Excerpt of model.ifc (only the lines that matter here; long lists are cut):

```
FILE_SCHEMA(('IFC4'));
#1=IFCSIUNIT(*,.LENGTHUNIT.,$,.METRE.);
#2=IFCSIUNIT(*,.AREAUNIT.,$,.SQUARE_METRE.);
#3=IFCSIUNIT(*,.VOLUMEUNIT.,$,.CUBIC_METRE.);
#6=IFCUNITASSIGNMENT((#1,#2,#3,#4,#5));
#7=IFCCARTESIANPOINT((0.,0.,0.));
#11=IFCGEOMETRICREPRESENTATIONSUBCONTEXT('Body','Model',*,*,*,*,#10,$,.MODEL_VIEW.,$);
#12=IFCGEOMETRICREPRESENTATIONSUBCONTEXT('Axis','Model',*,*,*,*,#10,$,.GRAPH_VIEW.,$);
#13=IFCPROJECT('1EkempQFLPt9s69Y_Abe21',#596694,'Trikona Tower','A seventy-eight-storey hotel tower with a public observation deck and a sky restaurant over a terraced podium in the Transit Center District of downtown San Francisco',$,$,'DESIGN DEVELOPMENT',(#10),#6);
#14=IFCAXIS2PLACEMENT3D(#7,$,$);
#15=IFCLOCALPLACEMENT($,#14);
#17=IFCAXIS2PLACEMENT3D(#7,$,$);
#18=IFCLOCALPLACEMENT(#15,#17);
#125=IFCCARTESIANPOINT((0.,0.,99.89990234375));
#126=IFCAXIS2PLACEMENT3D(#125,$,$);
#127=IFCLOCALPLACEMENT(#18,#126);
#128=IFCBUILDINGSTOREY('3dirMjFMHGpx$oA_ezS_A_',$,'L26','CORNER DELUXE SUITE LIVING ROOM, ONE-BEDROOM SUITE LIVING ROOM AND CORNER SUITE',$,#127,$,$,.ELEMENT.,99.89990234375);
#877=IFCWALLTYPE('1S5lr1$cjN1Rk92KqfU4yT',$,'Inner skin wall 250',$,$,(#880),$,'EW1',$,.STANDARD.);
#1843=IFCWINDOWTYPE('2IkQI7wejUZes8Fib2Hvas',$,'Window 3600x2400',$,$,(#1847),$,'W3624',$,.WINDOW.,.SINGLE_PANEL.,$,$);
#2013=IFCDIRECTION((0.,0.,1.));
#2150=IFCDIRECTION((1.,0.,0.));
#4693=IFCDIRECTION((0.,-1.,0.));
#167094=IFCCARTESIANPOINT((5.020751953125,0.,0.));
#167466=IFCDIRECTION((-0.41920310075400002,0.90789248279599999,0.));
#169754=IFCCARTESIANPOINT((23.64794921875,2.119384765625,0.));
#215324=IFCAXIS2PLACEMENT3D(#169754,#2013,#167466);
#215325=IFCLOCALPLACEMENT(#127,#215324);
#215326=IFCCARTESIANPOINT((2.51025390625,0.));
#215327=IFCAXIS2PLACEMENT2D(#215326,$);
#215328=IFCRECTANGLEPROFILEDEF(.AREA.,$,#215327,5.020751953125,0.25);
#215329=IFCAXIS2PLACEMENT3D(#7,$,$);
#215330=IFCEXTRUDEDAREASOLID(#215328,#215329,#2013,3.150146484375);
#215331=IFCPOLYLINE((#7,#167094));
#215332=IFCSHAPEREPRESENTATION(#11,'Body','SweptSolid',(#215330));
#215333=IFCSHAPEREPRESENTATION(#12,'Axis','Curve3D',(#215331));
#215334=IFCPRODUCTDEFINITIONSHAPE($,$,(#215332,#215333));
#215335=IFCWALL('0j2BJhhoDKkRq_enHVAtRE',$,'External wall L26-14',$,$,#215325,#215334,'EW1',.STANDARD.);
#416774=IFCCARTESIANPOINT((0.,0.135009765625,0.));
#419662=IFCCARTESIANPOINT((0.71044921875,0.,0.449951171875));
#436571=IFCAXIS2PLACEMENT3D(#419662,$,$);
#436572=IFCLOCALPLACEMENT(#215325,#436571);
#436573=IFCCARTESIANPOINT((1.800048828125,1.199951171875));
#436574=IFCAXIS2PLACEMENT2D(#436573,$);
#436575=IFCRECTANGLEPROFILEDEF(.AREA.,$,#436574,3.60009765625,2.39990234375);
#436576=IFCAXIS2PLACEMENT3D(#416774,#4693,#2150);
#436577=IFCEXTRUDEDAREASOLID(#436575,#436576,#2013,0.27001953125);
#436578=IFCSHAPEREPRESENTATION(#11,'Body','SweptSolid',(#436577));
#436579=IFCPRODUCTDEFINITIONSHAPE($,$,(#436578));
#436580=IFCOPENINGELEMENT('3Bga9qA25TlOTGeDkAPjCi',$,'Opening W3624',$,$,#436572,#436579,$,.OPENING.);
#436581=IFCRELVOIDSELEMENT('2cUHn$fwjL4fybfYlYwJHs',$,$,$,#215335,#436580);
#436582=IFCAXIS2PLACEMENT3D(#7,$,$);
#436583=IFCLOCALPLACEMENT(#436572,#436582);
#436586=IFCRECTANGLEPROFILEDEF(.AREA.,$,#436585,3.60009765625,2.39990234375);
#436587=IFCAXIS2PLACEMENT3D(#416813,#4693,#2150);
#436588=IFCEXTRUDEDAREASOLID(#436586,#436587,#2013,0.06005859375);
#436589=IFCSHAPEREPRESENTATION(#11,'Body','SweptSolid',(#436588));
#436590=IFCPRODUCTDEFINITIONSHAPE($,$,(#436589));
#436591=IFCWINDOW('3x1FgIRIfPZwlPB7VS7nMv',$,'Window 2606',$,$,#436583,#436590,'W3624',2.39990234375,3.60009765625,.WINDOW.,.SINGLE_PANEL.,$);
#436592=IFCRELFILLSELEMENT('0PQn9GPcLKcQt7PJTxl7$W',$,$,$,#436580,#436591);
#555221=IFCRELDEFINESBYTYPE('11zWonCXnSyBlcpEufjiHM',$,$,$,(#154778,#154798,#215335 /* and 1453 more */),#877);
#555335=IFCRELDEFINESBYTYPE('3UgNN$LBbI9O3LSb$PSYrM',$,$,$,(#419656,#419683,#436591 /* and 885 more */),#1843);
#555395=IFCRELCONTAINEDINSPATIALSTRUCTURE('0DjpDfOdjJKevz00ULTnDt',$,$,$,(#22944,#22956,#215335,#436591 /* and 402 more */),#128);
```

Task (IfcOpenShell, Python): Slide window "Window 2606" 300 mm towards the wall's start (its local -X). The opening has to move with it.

```python
import ifcopenshell
import ifcopenshell.api.geometry
import ifcopenshell.util.placement

model = ifcopenshell.open("model.ifc")

window = model.by_guid("3x1FgIRIfPZwlPB7VS7nMv")
opening = window.FillsVoids[0].RelatingOpeningElement
wall = opening.VoidsElements[0].RelatingBuildingElement

wall_matrix = ifcopenshell.util.placement.get_local_placement(wall.ObjectPlacement)
shift = wall_matrix[:3, 0] * -0.3
before = ifcopenshell.util.placement.get_local_placement(window.ObjectPlacement)[:3, 3].copy()

# The window is placed relative to its opening, so it follows when the opening moves.
matrix = ifcopenshell.util.placement.get_local_placement(opening.ObjectPlacement)
matrix[:3, 3] += shift
ifcopenshell.api.geometry.edit_object_placement(
    model, product=opening, matrix=matrix, is_si=False, should_transform_children=True
)

after = ifcopenshell.util.placement.get_local_placement(window.ObjectPlacement)[:3, 3]
print("window moved by", (after - before).round(3) + 0.0)

model.write("model-out.ifc")
```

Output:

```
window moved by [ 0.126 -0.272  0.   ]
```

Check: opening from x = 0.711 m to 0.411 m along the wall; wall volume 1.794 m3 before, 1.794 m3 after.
